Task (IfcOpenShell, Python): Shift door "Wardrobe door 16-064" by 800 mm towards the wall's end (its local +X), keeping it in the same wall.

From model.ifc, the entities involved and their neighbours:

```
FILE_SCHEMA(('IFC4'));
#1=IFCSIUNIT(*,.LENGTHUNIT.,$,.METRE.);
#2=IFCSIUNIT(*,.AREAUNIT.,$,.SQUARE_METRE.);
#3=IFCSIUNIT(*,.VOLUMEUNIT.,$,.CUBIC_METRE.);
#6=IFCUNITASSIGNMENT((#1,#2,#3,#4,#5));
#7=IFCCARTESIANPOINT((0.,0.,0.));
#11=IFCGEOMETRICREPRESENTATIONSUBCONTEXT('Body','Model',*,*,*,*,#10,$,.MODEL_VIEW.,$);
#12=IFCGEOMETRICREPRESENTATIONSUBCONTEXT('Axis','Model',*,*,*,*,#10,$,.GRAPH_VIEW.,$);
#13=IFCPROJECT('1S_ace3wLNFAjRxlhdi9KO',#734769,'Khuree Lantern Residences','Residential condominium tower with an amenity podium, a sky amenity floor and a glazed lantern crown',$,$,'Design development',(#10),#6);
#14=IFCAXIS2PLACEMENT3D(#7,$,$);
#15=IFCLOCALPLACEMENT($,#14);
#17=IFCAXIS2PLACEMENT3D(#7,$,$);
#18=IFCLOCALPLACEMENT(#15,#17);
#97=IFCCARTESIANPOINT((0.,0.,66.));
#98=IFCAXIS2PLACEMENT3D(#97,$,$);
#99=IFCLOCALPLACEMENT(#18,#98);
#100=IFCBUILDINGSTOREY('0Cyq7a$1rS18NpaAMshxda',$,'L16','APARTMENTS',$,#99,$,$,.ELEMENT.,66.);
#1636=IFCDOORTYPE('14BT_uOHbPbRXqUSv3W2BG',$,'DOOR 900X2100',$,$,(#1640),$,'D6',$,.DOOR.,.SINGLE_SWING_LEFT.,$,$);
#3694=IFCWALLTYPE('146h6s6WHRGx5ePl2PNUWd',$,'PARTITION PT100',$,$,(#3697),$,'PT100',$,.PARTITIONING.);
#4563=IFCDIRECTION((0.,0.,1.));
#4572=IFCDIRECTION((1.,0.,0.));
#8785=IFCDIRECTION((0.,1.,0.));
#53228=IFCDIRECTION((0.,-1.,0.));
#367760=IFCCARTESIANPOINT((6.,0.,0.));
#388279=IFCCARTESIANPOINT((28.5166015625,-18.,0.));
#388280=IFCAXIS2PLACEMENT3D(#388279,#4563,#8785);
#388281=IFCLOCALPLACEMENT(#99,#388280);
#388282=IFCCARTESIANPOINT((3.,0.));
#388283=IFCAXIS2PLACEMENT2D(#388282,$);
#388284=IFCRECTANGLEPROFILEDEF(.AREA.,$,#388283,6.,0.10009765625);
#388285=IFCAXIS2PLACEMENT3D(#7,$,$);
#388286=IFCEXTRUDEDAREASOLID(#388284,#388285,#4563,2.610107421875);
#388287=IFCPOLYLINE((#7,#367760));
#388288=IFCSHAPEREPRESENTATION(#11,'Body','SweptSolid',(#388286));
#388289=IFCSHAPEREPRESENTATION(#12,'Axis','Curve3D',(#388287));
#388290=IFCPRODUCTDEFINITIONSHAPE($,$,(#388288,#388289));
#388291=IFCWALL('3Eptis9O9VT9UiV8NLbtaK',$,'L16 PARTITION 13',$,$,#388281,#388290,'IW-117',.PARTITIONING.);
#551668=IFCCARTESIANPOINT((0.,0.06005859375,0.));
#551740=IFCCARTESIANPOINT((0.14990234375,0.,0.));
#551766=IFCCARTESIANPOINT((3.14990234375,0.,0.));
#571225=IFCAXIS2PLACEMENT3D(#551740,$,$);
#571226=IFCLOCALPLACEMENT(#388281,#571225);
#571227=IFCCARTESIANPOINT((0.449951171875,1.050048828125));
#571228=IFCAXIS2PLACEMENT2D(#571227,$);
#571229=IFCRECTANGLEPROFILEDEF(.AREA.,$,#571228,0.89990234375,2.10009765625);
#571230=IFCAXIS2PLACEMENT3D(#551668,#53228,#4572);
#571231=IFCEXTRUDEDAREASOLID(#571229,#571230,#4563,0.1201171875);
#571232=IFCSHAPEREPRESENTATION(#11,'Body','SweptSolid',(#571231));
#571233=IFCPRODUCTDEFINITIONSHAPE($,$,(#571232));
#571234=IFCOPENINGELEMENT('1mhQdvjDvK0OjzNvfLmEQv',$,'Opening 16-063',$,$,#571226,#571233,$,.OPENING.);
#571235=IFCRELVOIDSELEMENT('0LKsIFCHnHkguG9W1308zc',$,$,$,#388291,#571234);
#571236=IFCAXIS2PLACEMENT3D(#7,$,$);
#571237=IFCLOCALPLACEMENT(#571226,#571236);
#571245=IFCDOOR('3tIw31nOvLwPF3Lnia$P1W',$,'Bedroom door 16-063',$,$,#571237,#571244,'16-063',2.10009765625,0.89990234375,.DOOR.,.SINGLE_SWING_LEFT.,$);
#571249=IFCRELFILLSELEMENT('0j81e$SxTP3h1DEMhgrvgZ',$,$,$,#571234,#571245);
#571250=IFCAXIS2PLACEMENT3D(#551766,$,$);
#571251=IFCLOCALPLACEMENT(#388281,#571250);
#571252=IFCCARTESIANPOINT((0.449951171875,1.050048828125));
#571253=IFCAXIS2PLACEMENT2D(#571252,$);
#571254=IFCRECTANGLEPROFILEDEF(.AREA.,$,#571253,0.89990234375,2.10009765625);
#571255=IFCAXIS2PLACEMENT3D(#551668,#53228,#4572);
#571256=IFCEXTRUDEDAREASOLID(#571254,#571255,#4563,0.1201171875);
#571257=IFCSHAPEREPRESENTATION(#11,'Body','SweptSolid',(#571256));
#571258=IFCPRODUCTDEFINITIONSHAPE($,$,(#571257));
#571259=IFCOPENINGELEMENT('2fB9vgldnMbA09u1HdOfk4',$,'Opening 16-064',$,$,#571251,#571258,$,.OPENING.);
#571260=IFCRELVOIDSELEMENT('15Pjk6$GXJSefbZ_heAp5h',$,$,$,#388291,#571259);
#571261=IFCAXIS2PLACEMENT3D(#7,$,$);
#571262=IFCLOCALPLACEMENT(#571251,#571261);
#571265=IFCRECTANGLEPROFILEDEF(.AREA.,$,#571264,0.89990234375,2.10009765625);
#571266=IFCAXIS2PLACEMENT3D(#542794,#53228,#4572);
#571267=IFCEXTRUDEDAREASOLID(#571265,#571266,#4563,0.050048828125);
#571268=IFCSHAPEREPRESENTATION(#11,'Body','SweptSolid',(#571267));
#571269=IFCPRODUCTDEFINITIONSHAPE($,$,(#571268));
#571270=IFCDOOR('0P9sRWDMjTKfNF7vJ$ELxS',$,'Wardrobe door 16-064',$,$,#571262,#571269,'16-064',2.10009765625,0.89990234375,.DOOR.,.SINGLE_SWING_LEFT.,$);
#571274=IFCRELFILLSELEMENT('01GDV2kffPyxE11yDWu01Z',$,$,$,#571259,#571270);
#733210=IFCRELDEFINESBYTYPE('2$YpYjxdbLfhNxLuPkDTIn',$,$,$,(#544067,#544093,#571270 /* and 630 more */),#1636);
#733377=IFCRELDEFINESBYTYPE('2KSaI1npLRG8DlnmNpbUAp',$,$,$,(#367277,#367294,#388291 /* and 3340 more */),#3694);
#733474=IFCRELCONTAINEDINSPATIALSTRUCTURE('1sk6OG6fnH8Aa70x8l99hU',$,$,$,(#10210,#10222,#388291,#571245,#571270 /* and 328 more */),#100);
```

```python
import ifcopenshell
import ifcopenshell.api.geometry
import ifcopenshell.util.placement

model = ifcopenshell.open("model.ifc")

door = model.by_id(571270)
opening = door.FillsVoids[0].RelatingOpeningElement
wall = opening.VoidsElements[0].RelatingBuildingElement

wall_matrix = ifcopenshell.util.placement.get_local_placement(wall.ObjectPlacement)
shift = wall_matrix[:3, 0] * 0.8
before = ifcopenshell.util.placement.get_local_placement(door.ObjectPlacement)[:3, 3].copy()

# The door is placed relative to its opening, so it follows when the opening moves.
matrix = ifcopenshell.util.placement.get_local_placement(opening.ObjectPlacement)
matrix[:3, 3] += shift
ifcopenshell.api.geometry.edit_object_placement(
    model, product=opening, matrix=matrix, is_si=False, should_transform_children=True
)

after = ifcopenshell.util.placement.get_local_placement(door.ObjectPlacement)[:3, 3]
print("door moved by", (after - before).round(3) + 0.0)

model.write("model_v2.ifc")
```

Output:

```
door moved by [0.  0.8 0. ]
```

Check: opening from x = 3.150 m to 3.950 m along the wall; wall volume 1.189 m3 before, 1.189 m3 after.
